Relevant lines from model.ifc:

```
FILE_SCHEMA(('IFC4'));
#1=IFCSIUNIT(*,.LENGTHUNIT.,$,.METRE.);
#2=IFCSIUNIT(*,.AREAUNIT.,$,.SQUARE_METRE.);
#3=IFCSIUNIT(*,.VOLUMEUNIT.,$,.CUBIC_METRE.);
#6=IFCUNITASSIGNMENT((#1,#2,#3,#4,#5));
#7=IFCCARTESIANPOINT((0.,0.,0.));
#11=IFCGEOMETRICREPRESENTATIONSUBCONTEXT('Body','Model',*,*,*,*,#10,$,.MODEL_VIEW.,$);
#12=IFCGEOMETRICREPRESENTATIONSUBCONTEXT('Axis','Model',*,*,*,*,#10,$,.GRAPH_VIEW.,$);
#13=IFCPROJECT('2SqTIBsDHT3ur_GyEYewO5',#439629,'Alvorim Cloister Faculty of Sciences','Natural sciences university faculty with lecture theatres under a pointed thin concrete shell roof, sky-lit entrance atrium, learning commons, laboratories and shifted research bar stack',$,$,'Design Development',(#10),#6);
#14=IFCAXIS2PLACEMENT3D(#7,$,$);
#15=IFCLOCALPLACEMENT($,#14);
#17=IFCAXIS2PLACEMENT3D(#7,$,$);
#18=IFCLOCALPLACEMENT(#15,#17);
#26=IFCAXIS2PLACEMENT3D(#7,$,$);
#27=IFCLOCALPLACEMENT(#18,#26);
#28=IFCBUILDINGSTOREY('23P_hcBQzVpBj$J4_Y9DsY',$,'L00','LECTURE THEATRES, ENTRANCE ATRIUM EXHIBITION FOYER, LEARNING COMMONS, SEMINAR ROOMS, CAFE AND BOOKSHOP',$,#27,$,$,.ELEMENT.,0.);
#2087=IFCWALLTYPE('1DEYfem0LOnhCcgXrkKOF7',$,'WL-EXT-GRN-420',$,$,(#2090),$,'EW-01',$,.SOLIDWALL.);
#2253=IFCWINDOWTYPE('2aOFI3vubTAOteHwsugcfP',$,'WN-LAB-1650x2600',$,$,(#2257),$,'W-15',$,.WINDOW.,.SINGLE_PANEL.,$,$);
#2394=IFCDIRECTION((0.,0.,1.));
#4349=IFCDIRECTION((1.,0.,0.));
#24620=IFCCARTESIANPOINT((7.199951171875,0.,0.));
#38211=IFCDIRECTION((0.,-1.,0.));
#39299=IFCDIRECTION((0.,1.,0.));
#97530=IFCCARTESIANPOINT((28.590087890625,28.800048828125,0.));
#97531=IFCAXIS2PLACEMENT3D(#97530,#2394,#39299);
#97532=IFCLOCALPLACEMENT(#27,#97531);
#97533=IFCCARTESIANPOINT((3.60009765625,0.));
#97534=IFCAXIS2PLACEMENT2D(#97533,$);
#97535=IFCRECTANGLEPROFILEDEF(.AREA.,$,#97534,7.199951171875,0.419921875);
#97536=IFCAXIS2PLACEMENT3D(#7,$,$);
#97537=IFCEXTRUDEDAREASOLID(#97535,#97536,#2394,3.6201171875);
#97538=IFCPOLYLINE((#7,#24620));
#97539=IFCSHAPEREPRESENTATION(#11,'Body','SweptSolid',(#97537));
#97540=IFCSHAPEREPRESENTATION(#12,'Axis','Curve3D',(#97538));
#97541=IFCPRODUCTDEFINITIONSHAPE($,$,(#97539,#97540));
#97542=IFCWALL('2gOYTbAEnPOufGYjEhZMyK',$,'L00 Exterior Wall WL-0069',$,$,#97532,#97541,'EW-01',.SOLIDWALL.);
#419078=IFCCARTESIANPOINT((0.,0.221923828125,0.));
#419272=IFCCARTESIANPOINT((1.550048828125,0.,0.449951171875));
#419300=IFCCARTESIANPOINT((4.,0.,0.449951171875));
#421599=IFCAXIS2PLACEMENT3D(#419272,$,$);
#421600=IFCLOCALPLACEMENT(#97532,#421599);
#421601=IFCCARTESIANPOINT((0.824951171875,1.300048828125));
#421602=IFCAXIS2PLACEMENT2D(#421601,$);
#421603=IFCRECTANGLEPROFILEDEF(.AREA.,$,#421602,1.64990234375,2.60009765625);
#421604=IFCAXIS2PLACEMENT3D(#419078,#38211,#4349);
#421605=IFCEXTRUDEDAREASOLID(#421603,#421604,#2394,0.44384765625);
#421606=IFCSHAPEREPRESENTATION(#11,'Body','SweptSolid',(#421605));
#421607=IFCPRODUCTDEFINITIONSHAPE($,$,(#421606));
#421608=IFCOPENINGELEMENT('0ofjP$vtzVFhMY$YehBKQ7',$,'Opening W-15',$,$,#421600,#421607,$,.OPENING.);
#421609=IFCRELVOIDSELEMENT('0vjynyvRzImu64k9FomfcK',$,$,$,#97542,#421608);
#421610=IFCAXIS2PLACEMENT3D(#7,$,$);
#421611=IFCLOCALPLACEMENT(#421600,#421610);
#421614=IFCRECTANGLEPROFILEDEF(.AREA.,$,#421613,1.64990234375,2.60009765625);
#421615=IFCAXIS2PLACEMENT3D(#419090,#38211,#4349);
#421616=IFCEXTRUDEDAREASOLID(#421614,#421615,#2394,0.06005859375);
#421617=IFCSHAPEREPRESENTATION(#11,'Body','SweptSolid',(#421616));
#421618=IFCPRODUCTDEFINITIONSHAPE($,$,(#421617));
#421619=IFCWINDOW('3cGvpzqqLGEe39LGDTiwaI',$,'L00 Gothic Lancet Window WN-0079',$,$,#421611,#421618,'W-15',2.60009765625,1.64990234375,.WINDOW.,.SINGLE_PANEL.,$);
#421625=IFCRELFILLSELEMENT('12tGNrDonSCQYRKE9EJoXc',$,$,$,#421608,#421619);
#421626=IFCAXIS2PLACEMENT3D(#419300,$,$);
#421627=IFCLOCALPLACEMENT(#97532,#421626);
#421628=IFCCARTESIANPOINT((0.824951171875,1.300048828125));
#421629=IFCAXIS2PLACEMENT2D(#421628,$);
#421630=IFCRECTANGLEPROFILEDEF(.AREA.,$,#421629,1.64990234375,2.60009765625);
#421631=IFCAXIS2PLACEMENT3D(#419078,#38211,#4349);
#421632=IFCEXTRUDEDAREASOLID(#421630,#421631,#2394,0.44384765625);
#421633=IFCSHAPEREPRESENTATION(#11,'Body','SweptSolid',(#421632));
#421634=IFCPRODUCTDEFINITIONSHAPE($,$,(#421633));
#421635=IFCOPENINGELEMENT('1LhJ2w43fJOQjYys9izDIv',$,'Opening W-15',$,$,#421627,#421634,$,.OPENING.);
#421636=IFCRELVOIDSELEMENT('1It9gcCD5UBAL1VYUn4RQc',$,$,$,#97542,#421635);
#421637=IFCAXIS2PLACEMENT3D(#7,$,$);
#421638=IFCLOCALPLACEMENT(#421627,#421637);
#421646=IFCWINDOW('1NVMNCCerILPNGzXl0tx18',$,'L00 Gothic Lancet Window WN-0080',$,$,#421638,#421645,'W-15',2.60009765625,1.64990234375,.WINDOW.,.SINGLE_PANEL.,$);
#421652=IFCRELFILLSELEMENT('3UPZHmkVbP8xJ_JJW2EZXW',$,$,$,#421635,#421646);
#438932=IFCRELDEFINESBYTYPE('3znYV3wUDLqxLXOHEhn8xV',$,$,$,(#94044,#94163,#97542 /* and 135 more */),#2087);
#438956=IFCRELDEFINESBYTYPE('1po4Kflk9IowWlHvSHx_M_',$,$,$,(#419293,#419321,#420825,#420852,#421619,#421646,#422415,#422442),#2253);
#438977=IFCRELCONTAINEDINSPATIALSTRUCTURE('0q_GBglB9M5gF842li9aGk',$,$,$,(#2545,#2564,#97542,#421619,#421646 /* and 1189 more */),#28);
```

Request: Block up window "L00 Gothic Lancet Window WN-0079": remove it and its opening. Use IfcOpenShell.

```python
import ifcopenshell
import ifcopenshell.api.feature
import ifcopenshell.api.root
import ifcopenshell.geom
import ifcopenshell.util.shape

model = ifcopenshell.open("model.ifc")
settings = ifcopenshell.geom.settings()


def volume(element):
    """Net volume in cubic metres, openings subtracted."""
    shape = ifcopenshell.geom.create_shape(settings, element)
    return ifcopenshell.util.shape.get_volume(shape.geometry)


window = model.by_guid("3cGvpzqqLGEe39LGDTiwaI")
opening = window.FillsVoids[0].RelatingOpeningElement
wall = opening.VoidsElements[0].RelatingBuildingElement
before = volume(wall)

ifcopenshell.api.root.remove_product(model, product=window)
ifcopenshell.api.feature.remove_feature(model, feature=opening)

after = volume(wall)

print(f"wall volume {before:.3f} -> {after:.3f} m3")

model.write("model-out.ifc")
```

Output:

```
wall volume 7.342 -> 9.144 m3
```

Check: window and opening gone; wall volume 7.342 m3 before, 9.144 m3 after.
